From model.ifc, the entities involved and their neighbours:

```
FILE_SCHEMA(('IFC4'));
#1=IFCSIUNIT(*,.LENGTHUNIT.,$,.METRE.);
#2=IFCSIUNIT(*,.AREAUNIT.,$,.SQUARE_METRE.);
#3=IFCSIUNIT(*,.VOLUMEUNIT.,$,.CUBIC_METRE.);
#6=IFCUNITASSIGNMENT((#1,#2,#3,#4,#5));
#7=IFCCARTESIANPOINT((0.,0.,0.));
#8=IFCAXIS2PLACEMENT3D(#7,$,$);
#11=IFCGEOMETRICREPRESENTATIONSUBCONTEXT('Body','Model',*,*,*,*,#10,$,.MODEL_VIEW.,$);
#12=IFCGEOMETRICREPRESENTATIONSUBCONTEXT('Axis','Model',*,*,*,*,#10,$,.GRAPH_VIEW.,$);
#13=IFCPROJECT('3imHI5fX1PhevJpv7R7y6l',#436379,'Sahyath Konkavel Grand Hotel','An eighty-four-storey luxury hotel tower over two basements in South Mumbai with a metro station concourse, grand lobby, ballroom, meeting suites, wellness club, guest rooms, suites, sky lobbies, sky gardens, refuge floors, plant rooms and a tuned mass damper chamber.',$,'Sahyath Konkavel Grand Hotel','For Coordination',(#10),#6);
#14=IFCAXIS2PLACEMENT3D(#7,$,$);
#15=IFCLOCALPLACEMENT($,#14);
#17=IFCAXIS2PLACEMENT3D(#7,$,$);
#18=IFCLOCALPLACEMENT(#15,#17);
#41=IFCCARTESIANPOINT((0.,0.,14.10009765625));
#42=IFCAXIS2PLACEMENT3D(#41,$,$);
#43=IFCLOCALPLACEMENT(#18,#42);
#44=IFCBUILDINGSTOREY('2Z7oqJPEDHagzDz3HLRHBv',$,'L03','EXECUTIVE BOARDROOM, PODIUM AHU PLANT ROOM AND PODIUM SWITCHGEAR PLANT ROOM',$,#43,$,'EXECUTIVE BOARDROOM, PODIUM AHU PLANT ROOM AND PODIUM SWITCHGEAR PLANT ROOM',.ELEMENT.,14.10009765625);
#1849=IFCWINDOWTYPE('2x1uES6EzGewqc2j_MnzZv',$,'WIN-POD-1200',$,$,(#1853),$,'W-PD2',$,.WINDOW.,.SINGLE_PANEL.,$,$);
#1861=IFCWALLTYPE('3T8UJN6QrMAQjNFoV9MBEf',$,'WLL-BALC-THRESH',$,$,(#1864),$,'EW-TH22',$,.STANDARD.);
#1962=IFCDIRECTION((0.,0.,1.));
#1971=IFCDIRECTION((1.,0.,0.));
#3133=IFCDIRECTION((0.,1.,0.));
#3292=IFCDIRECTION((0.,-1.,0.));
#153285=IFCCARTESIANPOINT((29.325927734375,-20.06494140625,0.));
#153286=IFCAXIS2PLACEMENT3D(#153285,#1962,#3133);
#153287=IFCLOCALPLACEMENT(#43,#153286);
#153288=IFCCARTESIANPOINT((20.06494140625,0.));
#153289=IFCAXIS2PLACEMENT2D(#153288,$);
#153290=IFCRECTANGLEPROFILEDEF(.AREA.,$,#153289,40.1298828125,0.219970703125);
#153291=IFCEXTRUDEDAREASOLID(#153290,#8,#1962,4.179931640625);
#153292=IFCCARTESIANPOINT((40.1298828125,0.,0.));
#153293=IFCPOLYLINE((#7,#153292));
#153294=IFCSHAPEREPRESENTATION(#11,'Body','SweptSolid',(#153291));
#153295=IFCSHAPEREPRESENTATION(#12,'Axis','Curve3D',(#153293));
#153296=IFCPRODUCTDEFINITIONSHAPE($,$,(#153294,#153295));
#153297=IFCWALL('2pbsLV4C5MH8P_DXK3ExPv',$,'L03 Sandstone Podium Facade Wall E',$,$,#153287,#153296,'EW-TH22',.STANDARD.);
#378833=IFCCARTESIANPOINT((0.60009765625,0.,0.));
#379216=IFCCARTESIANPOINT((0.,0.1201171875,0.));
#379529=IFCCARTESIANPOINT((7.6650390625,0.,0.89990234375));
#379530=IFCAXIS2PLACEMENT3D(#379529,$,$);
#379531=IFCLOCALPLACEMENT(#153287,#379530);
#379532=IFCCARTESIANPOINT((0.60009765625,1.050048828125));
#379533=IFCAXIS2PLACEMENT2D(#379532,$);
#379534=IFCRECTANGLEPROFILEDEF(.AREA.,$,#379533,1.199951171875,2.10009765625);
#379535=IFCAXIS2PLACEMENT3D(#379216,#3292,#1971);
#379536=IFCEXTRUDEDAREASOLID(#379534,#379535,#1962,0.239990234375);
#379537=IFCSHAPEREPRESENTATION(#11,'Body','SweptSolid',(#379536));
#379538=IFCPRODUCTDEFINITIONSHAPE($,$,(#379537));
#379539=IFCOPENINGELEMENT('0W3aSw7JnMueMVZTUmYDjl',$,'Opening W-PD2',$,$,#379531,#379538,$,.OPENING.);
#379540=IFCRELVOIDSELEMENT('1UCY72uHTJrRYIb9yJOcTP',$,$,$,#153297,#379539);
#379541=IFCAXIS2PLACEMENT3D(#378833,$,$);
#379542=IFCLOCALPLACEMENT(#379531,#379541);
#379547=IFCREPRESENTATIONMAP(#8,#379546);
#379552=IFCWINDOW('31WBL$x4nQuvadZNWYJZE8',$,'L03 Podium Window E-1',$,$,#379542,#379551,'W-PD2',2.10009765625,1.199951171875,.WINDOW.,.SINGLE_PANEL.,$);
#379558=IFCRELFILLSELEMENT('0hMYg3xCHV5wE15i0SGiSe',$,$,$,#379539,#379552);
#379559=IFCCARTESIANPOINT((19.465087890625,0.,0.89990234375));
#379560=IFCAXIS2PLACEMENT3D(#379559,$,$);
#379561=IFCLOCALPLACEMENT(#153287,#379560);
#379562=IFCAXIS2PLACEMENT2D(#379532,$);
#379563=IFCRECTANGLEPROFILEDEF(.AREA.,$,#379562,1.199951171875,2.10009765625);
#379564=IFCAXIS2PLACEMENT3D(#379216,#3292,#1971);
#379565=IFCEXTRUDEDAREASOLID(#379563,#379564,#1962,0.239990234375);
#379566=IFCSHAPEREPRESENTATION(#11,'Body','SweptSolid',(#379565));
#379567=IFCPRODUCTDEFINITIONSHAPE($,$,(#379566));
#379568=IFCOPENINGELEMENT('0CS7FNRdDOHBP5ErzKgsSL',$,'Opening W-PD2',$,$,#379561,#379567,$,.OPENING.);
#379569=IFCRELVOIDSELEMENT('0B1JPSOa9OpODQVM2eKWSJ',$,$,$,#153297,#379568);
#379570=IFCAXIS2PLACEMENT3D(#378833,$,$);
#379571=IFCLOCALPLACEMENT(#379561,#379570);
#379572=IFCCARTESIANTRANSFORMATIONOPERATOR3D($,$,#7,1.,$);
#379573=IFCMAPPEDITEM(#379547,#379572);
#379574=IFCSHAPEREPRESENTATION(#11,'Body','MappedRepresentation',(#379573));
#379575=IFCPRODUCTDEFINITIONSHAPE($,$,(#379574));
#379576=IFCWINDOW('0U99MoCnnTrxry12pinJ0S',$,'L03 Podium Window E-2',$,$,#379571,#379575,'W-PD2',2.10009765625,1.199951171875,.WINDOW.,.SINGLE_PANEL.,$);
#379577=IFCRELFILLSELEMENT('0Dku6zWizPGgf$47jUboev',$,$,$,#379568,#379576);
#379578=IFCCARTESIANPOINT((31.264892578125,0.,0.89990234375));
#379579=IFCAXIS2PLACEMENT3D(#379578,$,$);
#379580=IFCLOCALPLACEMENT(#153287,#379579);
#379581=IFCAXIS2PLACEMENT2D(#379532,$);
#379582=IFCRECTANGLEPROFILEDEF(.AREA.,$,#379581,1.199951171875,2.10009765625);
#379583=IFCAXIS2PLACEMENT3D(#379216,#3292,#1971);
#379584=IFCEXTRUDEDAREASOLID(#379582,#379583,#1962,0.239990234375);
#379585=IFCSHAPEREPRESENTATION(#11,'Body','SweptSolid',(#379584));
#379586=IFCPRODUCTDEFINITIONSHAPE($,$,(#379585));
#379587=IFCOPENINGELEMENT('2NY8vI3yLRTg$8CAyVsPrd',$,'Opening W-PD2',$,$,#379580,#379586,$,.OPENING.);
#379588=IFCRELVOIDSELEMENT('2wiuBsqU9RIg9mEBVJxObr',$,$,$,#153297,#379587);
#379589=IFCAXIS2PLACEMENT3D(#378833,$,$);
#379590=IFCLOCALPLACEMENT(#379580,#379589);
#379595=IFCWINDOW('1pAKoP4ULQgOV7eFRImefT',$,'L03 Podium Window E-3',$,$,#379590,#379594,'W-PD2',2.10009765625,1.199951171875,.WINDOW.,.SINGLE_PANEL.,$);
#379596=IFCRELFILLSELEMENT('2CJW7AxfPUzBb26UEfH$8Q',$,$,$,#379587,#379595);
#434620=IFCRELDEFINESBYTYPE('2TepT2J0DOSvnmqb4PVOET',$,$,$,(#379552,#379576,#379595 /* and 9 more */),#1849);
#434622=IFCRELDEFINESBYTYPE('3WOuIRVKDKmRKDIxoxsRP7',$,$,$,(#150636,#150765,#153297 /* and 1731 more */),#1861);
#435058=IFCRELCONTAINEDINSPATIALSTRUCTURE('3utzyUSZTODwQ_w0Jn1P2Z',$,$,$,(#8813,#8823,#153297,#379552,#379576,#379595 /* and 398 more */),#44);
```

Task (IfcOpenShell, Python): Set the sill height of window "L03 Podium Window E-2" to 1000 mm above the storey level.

```python
import numpy as np
import ifcopenshell
import ifcopenshell.api.geometry
import ifcopenshell.geom
import ifcopenshell.util.element
import ifcopenshell.util.placement
import ifcopenshell.util.shape
import ifcopenshell.util.unit

model = ifcopenshell.open("model.ifc")
unit_scale = ifcopenshell.util.unit.calculate_unit_scale(model)

window = model.by_id(379576)
opening = window.FillsVoids[0].RelatingOpeningElement
storey = ifcopenshell.util.element.get_container(window, ifc_class="IfcBuildingStorey")
level = ifcopenshell.util.placement.get_local_placement(storey.ObjectPlacement)[2, 3]

# The opening's origin need not be at the sill, so measure its lowest point.
shape = ifcopenshell.geom.create_shape(ifcopenshell.geom.settings(), opening)
bottom = ifcopenshell.util.shape.get_shape_bottom_elevation(shape, shape.geometry) / unit_scale
dz = level + 1 / unit_scale - bottom

shift = np.array([0.0, 0.0, dz])
# The window is placed relative to its opening, so it follows when the opening moves.
matrix = ifcopenshell.util.placement.get_local_placement(opening.ObjectPlacement)
matrix[:3, 3] += shift
ifcopenshell.api.geometry.edit_object_placement(
    model, product=opening, matrix=matrix, is_si=False, should_transform_children=True
)

print(f"moved by {dz * unit_scale:+.3f} m")

model.write("model_updated.ifc")
```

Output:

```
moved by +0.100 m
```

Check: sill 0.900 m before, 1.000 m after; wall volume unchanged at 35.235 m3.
